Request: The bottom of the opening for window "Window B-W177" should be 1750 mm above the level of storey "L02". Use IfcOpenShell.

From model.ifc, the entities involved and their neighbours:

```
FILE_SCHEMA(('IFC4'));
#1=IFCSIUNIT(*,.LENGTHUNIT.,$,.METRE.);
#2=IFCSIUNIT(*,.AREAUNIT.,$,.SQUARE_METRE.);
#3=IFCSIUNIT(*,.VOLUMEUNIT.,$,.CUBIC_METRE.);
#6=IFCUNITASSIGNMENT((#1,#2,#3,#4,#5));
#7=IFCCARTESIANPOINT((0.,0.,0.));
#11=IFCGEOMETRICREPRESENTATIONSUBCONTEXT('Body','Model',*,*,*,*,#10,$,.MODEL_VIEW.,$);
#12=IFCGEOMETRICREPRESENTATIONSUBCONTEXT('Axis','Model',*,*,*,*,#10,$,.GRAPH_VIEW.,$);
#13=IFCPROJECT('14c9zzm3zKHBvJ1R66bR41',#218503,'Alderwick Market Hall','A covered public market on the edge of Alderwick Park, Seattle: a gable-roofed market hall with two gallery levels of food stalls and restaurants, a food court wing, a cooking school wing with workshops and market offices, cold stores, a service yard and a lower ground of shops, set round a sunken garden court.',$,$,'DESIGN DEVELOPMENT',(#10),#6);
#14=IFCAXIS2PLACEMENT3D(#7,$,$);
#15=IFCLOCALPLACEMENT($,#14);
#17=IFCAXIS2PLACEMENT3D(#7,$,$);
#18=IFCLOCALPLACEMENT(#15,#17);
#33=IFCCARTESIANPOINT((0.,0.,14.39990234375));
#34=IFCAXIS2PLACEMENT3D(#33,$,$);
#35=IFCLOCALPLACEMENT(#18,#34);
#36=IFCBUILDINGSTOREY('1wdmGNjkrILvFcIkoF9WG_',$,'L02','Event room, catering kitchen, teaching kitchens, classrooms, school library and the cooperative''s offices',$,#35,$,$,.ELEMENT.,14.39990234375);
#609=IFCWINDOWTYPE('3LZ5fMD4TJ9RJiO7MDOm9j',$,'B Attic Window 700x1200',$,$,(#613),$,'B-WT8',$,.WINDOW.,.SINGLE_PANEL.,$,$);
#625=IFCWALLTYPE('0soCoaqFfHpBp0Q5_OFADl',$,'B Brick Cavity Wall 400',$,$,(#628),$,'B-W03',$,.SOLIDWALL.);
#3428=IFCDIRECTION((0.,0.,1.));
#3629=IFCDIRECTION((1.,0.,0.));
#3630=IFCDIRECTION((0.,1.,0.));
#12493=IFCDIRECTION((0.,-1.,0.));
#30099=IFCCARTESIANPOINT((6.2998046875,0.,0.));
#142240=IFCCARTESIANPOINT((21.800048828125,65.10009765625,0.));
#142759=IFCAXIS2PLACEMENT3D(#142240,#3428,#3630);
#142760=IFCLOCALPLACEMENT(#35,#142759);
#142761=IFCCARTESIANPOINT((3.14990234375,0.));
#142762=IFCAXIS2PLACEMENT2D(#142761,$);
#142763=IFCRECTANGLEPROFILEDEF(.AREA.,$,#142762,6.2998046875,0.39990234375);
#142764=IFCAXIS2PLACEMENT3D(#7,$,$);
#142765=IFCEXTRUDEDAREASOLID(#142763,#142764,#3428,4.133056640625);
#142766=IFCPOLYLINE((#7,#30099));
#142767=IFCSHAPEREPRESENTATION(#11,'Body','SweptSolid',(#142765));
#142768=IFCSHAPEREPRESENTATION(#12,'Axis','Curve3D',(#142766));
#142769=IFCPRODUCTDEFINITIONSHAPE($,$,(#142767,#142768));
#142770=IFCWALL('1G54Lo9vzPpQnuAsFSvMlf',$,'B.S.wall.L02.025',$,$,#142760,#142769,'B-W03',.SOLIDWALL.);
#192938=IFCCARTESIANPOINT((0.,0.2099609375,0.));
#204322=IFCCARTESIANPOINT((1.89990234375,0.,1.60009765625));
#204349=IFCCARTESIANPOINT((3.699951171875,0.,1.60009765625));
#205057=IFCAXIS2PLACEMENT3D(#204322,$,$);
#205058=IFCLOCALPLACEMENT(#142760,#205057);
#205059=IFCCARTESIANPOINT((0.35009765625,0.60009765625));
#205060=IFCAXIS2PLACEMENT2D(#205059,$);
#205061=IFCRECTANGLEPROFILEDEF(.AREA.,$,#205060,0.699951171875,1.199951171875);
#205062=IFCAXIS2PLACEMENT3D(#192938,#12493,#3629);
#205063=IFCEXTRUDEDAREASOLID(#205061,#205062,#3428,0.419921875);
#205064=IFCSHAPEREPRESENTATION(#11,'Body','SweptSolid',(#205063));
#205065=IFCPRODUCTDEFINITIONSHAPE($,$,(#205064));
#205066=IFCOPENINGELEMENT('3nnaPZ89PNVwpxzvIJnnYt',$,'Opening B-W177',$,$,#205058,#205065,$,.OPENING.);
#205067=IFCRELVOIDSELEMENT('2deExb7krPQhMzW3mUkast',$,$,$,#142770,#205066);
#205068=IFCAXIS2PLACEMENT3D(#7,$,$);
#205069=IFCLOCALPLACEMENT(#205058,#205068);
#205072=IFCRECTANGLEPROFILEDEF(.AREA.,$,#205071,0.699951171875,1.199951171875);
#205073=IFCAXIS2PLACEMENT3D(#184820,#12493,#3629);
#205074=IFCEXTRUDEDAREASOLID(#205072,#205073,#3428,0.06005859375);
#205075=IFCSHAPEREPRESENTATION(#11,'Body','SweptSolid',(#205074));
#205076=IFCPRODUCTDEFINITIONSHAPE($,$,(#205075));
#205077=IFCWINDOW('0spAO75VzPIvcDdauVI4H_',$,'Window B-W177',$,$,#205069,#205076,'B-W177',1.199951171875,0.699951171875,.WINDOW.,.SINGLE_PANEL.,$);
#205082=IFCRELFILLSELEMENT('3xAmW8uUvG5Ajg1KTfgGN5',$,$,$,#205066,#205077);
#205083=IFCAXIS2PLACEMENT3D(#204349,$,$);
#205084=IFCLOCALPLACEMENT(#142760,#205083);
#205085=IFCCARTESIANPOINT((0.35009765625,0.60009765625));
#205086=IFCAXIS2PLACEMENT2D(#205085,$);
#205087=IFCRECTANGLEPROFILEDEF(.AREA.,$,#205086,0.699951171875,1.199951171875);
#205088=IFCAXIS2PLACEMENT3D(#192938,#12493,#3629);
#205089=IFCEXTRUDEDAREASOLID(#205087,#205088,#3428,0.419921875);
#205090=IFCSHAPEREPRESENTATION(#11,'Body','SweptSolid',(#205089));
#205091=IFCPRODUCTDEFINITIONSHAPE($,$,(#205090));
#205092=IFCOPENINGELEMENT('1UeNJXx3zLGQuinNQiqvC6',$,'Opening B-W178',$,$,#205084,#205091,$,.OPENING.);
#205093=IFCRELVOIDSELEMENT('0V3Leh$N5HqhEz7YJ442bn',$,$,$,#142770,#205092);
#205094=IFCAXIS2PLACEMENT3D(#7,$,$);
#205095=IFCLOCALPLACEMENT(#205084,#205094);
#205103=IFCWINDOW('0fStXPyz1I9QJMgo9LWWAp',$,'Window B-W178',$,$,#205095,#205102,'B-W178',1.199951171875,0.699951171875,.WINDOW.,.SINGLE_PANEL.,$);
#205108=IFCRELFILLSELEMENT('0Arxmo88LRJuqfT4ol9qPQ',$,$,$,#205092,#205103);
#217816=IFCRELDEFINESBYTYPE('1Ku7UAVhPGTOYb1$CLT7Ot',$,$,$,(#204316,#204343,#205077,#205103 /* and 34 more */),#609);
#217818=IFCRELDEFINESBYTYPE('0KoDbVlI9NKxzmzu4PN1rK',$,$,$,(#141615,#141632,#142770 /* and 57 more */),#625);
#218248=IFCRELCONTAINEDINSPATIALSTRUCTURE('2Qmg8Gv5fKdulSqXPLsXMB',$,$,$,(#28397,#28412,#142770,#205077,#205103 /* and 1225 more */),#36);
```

```python
import numpy as np
import ifcopenshell
import ifcopenshell.api.geometry
import ifcopenshell.geom
import ifcopenshell.util.element
import ifcopenshell.util.placement
import ifcopenshell.util.shape
import ifcopenshell.util.unit

model = ifcopenshell.open("model.ifc")
unit_scale = ifcopenshell.util.unit.calculate_unit_scale(model)

window = model.by_guid("0spAO75VzPIvcDdauVI4H_")
opening = window.FillsVoids[0].RelatingOpeningElement
storey = ifcopenshell.util.element.get_container(window, ifc_class="IfcBuildingStorey")
level = ifcopenshell.util.placement.get_local_placement(storey.ObjectPlacement)[2, 3]

# The opening's origin need not be at the sill, so measure its lowest point.
shape = ifcopenshell.geom.create_shape(ifcopenshell.geom.settings(), opening)
bottom = ifcopenshell.util.shape.get_shape_bottom_elevation(shape, shape.geometry) / unit_scale
dz = level + 1.75 / unit_scale - bottom

shift = np.array([0.0, 0.0, dz])
# The window is placed relative to its opening, so it follows when the opening moves.
matrix = ifcopenshell.util.placement.get_local_placement(opening.ObjectPlacement)
matrix[:3, 3] += shift
ifcopenshell.api.geometry.edit_object_placement(
    model, product=opening, matrix=matrix, is_si=False, should_transform_children=True
)

print(f"moved by {dz * unit_scale:+.3f} m")

model.write("model_rev.ifc")
```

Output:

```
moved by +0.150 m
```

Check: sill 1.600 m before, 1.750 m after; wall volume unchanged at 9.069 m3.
